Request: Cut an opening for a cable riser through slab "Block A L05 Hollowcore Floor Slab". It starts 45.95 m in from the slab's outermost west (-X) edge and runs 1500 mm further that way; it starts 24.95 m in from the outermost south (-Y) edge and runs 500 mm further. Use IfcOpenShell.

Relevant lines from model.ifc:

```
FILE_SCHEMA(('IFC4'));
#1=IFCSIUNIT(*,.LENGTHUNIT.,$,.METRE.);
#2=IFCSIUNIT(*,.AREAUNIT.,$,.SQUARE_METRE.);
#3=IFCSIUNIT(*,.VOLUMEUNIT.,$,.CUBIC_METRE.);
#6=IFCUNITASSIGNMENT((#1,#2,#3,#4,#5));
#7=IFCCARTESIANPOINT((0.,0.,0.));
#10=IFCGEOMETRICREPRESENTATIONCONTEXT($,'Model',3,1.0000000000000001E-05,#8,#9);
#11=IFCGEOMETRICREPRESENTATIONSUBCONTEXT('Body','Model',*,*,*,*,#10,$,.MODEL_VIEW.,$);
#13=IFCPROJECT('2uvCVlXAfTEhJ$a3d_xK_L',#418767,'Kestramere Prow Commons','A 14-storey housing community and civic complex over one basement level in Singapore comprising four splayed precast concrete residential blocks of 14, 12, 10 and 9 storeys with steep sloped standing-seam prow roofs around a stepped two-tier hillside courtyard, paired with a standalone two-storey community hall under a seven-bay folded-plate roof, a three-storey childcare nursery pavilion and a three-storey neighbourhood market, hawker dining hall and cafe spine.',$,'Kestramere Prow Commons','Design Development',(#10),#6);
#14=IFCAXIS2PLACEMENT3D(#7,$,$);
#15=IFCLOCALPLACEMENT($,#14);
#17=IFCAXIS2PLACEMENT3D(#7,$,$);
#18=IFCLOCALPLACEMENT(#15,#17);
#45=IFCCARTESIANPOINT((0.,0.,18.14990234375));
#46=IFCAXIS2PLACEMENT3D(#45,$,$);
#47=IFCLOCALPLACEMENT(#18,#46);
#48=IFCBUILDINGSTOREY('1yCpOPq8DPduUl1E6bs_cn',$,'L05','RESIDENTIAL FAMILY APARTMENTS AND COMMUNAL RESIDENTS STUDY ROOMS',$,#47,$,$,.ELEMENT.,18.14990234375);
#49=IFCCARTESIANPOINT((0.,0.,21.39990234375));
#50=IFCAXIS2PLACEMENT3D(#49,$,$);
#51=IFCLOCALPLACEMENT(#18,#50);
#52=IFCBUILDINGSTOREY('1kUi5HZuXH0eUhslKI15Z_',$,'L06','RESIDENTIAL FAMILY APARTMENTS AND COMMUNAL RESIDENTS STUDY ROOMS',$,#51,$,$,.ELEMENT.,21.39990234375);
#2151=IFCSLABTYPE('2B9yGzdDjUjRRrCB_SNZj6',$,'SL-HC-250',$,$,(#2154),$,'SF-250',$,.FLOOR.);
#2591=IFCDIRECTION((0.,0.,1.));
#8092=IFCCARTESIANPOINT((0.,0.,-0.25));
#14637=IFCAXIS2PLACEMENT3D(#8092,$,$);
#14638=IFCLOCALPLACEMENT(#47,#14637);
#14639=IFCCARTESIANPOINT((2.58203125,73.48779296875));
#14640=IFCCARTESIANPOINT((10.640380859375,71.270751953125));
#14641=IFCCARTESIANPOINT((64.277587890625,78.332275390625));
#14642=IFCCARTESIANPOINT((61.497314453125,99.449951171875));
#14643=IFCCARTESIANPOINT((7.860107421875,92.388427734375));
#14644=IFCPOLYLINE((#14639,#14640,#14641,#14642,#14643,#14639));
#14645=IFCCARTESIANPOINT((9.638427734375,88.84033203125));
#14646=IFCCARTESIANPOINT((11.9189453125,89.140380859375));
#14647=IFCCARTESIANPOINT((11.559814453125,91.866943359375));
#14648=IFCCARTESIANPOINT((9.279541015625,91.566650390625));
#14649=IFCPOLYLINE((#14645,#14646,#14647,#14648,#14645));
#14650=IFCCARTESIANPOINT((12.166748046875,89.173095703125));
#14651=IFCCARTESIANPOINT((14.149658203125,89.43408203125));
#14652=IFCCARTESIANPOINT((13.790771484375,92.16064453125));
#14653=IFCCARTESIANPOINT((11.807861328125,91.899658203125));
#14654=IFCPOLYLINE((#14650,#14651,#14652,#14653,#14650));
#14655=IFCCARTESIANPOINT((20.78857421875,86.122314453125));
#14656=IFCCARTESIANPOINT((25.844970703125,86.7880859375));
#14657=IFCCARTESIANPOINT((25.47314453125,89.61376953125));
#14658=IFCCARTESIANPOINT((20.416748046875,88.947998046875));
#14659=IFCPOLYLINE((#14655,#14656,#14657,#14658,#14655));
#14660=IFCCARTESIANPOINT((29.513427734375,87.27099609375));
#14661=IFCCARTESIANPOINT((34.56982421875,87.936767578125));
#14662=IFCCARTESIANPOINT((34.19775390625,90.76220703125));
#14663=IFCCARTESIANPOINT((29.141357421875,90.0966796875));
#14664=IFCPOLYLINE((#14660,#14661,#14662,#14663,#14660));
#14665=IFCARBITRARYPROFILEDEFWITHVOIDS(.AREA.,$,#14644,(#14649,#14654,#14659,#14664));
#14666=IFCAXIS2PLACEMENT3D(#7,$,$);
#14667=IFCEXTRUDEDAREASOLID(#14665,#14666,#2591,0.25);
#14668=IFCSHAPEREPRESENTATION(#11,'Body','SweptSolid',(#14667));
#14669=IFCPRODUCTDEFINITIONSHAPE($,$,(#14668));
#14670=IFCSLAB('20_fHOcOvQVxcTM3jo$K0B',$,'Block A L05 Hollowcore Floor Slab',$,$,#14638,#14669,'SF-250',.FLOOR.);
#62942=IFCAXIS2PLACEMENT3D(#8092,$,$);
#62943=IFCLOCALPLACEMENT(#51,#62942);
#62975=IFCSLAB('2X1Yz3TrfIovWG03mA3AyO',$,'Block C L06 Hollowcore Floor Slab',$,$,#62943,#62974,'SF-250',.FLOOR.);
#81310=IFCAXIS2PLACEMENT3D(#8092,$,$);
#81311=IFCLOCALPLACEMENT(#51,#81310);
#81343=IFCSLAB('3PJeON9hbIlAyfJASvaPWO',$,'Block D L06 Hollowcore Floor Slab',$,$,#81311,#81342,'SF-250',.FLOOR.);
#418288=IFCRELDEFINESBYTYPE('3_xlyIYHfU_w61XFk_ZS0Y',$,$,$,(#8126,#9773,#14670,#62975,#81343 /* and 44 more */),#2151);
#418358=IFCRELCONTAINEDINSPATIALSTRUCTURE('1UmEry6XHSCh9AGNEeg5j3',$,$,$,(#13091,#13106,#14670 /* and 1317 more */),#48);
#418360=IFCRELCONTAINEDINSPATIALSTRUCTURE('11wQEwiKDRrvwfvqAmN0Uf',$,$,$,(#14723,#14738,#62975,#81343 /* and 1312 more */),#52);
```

```python
import numpy as np
import ifcopenshell
import ifcopenshell.api.feature
import ifcopenshell.api.geometry
import ifcopenshell.api.root
import ifcopenshell.geom
import ifcopenshell.util.placement
import ifcopenshell.util.representation
import ifcopenshell.util.shape
import ifcopenshell.util.unit

model = ifcopenshell.open("model.ifc")
unit_scale = ifcopenshell.util.unit.calculate_unit_scale(model)
settings = ifcopenshell.geom.settings()


def volume(element):
    """Net volume in cubic metres, openings subtracted."""
    shape = ifcopenshell.geom.create_shape(settings, element)
    return ifcopenshell.util.shape.get_volume(shape.geometry)


slab = model.by_id(14670)
before = volume(slab)

# Extent in the slab's own axes, in metres. The edges named are its -X and -Y sides.
slab_shape = ifcopenshell.geom.create_shape(settings, slab)
vertices = ifcopenshell.util.shape.get_vertices(slab_shape.geometry)
x_min, y_min, bottom = vertices.min(axis=0)
top = vertices[:, 2].max()

opening = ifcopenshell.api.root.create_entity(model, ifc_class="IfcOpeningElement", name="Cable riser opening", predefined_type="OPENING")
context = ifcopenshell.util.representation.get_context(model, "Model", "Body", "MODEL_VIEW")
width, depth = 1.5, 0.5
outline = [(0.0, 0.0), (width, 0.0), (width, depth), (0.0, depth), (0.0, 0.0)]
# Overshoot both faces by 50 mm so the cut is clean.
shape = ifcopenshell.api.geometry.add_slab_representation(
    model, context=context, depth=top - bottom + 0.1, polyline=outline
)
ifcopenshell.api.geometry.assign_representation(model, product=opening, representation=shape)

matrix = ifcopenshell.util.placement.get_local_placement(slab.ObjectPlacement)
matrix[:, 3] = matrix @ np.append(np.array([x_min + 45.95, y_min + 24.95, bottom - 0.05]) / unit_scale, 1.0)
ifcopenshell.api.geometry.edit_object_placement(model, product=opening, matrix=matrix, is_si=False)
ifcopenshell.api.feature.add_feature(model, feature=opening, element=slab)

after = volume(slab)

print(f"slab volume {before:.3f} -> {after:.3f} m3")

model.write("model_v2.ifc")
```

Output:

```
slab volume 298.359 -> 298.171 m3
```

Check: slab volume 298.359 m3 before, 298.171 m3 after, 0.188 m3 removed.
